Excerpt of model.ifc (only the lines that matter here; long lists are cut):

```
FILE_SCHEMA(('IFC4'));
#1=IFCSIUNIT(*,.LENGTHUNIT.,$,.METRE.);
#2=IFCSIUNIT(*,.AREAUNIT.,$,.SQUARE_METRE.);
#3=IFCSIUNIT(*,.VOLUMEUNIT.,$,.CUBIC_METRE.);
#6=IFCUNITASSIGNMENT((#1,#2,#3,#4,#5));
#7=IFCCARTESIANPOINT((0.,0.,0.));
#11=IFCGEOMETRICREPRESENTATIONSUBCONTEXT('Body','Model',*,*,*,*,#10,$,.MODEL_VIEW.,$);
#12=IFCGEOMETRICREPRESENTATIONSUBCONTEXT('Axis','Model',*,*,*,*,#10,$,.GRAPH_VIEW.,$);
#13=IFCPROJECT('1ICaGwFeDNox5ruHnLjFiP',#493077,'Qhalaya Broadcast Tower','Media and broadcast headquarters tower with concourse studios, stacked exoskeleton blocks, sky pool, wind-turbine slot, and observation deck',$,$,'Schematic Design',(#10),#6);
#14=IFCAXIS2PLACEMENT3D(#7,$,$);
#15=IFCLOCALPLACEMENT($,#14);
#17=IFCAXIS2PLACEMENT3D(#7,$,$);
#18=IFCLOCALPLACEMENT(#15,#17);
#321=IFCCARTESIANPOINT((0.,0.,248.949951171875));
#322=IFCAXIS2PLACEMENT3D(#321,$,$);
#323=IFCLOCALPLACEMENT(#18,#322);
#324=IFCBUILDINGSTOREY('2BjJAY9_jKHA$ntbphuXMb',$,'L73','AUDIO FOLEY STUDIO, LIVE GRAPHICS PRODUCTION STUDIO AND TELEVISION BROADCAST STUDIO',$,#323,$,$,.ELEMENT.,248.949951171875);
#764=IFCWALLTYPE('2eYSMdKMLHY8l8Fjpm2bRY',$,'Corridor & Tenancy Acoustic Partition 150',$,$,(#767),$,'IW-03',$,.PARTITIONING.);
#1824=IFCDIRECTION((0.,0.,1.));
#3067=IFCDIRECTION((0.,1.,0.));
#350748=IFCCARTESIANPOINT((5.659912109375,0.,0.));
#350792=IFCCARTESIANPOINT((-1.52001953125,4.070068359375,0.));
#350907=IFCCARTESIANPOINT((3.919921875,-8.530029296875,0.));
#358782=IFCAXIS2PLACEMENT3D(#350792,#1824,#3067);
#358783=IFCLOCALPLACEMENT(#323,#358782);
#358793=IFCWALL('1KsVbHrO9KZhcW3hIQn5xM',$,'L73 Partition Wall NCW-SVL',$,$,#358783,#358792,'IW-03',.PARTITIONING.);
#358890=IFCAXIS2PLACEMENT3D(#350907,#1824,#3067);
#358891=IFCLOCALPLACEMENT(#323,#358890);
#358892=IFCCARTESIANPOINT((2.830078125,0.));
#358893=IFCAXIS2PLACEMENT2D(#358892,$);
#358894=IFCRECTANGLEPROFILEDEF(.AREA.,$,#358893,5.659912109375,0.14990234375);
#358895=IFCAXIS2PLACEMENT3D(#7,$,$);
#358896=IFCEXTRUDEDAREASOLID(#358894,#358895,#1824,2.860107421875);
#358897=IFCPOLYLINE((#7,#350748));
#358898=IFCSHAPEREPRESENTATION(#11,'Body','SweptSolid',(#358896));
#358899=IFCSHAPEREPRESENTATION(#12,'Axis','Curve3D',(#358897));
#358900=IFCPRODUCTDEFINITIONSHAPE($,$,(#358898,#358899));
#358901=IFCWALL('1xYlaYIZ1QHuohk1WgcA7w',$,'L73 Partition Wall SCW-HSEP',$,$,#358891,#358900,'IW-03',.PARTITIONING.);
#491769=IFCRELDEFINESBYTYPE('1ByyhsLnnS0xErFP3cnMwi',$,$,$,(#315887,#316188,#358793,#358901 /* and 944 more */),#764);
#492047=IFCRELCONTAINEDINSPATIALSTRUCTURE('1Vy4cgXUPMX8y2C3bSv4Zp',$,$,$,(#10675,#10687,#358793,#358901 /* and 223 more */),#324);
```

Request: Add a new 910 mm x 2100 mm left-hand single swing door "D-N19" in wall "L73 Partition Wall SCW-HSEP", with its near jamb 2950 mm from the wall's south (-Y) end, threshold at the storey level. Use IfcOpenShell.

```python
import numpy as np
import ifcopenshell
import ifcopenshell.api.feature
import ifcopenshell.api.geometry
import ifcopenshell.api.root
import ifcopenshell.api.spatial
import ifcopenshell.geom
import ifcopenshell.util.element
import ifcopenshell.util.placement
import ifcopenshell.util.representation
import ifcopenshell.util.shape
import ifcopenshell.util.unit

model = ifcopenshell.open("model.ifc")
unit_scale = ifcopenshell.util.unit.calculate_unit_scale(model)
settings = ifcopenshell.geom.settings()


def volume(element):
    """Net volume in cubic metres, openings subtracted."""
    shape = ifcopenshell.geom.create_shape(settings, element)
    return ifcopenshell.util.shape.get_volume(shape.geometry)


wall = model.by_guid("1xYlaYIZ1QHuohk1WgcA7w")
storey = ifcopenshell.util.element.get_container(wall, ifc_class="IfcBuildingStorey")
context = ifcopenshell.util.representation.get_context(model, "Model", "Body", "MODEL_VIEW")
before = volume(wall)

width, height, from_end, sill = 0.91, 2.1, 2.95, 0.0  # metres

# The wall runs along its own X axis, and the end named is its -X end.
wall_shape = ifcopenshell.geom.create_shape(settings, wall)
x, y, z = ifcopenshell.util.shape.get_vertices(wall_shape.geometry).T
start = x.min() + from_end
face, thickness = float(y.min()), float(y.max() - y.min())
wall_matrix = ifcopenshell.util.placement.get_local_placement(wall.ObjectPlacement)
level = ifcopenshell.util.placement.get_local_placement(storey.ObjectPlacement)[2, 3]


def in_wall(x, y):
    """Placement at x, y metres in the wall's axes, at sill height."""
    matrix = wall_matrix.copy()
    matrix[:, 3] = wall_matrix @ np.array([x / unit_scale, y / unit_scale, 0.0, 1.0])
    matrix[2, 3] = level + sill / unit_scale
    return matrix


# Opening: a box that overshoots both wall faces by 50 mm.
opening = ifcopenshell.api.root.create_entity(model, ifc_class="IfcOpeningElement", predefined_type="OPENING")
box = ifcopenshell.api.geometry.add_wall_representation(
    model, context=context, length=width, height=height, thickness=thickness + 0.1
)
ifcopenshell.api.geometry.assign_representation(model, product=opening, representation=box)
ifcopenshell.api.geometry.edit_object_placement(model, product=opening, matrix=in_wall(start, face - 0.05), is_si=False)
ifcopenshell.api.feature.add_feature(model, feature=opening, element=wall)

door = ifcopenshell.api.root.create_entity(model, ifc_class="IfcDoor", name="D-N19", predefined_type="DOOR")
door.OverallWidth, door.OverallHeight = width / unit_scale, height / unit_scale
door.OperationType = "SINGLE_SWING_LEFT"
body = ifcopenshell.api.geometry.add_door_representation(
    model,
    context=context,
    overall_width=door.OverallWidth,
    overall_height=door.OverallHeight,
    operation_type="SINGLE_SWING_LEFT",
    lining_properties={"LiningDepth": thickness / unit_scale, "ThresholdDepth": thickness / unit_scale},
)
ifcopenshell.api.geometry.assign_representation(model, product=door, representation=body)
ifcopenshell.api.spatial.assign_container(model, products=[door], relating_structure=storey)
ifcopenshell.api.feature.add_filling(model, opening=opening, element=door)

# The lining spans the wall, so the door starts at the wall face.
ifcopenshell.api.geometry.edit_object_placement(model, product=door, matrix=in_wall(start, face), is_si=False)

after = volume(wall)

print(f"wall volume {before:.3f} -> {after:.3f} m3")

model.write("model-out.ifc")
```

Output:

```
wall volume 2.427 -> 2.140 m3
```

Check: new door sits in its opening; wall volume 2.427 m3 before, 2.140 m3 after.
